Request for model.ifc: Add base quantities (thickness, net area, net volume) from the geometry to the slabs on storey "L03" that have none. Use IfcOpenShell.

First a look at what the model holds.

```python
import ifcopenshell
import ifcopenshell.util.element
import ifcopenshell.util.unit

model = ifcopenshell.open("model.ifc")
print(model.schema)
for unit_type in ("LENGTHUNIT", "AREAUNIT", "VOLUMEUNIT"):
    print(unit_type, ifcopenshell.util.unit.calculate_unit_scale(model, unit_type))
storey = next(s for s in model.by_type("IfcBuildingStorey") if s.Name == "L03")
slabs = [e for e in ifcopenshell.util.element.get_decomposition(storey) if e.is_a("IfcSlab")]
for e in sorted(slabs, key=lambda e: e.id()):
    print(e.id(), e.is_a(), e.Name, list(ifcopenshell.util.element.get_psets(e, qtos_only=True)), sep=" | ")
```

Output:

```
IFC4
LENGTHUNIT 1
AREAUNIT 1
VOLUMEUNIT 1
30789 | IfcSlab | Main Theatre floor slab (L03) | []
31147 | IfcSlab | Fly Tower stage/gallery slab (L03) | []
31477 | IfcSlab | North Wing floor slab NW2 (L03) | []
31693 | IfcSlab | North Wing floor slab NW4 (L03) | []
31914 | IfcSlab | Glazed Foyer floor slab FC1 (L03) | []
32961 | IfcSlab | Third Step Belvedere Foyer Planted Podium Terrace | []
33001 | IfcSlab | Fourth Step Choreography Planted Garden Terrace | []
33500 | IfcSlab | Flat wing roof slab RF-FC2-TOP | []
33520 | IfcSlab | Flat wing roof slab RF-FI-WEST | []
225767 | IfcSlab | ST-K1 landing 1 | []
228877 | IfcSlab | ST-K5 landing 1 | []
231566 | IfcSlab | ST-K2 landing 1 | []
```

```python
import ifcopenshell
import ifcopenshell.api.pset
import ifcopenshell.geom
import ifcopenshell.util.element
import ifcopenshell.util.shape
import ifcopenshell.util.unit

model = ifcopenshell.open("model.ifc")
unit_scale = ifcopenshell.util.unit.calculate_unit_scale(model)
area_scale = ifcopenshell.util.unit.calculate_unit_scale(model, "AREAUNIT")
volume_scale = ifcopenshell.util.unit.calculate_unit_scale(model, "VOLUMEUNIT")
settings = ifcopenshell.geom.settings()

storey = next(s for s in model.by_type("IfcBuildingStorey") if s.Name == "L03")
slabs = [e for e in ifcopenshell.util.element.get_decomposition(storey) if e.is_a("IfcSlab")]

for e in sorted(slabs, key=lambda e: e.id()):
    if ifcopenshell.util.element.get_psets(e, qtos_only=True, should_inherit=False):
        continue
    # Geometry comes back in metres, in the element's own axes.
    shape = ifcopenshell.geom.create_shape(settings, e)
    values = {
        "Width": ifcopenshell.util.shape.get_z(shape.geometry) / unit_scale,
        "NetArea": ifcopenshell.util.shape.get_footprint_area(shape.geometry) / area_scale,
        "NetVolume": ifcopenshell.util.shape.get_volume(shape.geometry) / volume_scale,
    }
    qto = ifcopenshell.api.pset.add_qto(model, product=e, name="Qto_SlabBaseQuantities")
    ifcopenshell.api.pset.edit_qto(model, qto=qto, properties=values)
    print(e.id(), {k: round(v, 3) for k, v in values.items()})

model.write("model_v2.ifc")
```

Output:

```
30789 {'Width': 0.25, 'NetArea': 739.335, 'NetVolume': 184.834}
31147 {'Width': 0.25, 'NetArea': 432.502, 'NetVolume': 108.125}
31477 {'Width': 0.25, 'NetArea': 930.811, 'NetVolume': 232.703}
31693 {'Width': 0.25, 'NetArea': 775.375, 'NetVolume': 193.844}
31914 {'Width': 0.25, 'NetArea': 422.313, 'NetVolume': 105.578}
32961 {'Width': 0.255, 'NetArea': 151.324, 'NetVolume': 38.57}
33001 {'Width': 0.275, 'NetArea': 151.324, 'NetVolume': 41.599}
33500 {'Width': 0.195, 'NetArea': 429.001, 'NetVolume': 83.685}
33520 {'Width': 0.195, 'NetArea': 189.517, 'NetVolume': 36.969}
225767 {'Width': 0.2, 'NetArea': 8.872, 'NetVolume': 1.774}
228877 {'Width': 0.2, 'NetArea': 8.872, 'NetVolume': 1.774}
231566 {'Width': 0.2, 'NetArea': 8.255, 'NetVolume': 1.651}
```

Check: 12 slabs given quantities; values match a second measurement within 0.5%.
